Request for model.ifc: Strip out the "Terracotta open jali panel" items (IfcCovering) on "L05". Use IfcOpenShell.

First a look at what the model holds.

```python
import ifcopenshell
import ifcopenshell.util.element

model = ifcopenshell.open("model.ifc")
print(model.schema)
storey = next(s for s in model.by_type("IfcBuildingStorey") if s.Name == "L05")
coverings = [e for e in ifcopenshell.util.element.get_decomposition(storey) if e.is_a("IfcCovering")]
seen = {}
for e in coverings:
    element_type = ifcopenshell.util.element.get_type(e)
    name = element_type.Name if element_type not in (None, e) else None
    seen[name] = seen.get(name, 0) + 1
for name, count in sorted(seen.items(), key=str):
    print(count, "x", name)
```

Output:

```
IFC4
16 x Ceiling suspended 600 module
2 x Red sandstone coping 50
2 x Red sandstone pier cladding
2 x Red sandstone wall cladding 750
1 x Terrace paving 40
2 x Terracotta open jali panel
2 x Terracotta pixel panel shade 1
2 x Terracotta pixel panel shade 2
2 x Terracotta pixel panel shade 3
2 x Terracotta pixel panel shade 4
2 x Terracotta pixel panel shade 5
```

```python
import ifcopenshell
import ifcopenshell.api.root
import ifcopenshell.util.element

model = ifcopenshell.open("model.ifc")

storey = next(s for s in model.by_type("IfcBuildingStorey") if s.Name == "L05")
coverings = [e for e in ifcopenshell.util.element.get_decomposition(storey) if e.is_a("IfcCovering")]
targets = [e for e in coverings if (t := ifcopenshell.util.element.get_type(e)) not in (None, e) and t.Name == "Terracotta open jali panel"]

for e in targets:
    ifcopenshell.api.root.remove_product(model, product=e)
print(len(targets), "removed")

model.write("model_edited.ifc")
```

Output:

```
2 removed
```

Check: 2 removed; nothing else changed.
